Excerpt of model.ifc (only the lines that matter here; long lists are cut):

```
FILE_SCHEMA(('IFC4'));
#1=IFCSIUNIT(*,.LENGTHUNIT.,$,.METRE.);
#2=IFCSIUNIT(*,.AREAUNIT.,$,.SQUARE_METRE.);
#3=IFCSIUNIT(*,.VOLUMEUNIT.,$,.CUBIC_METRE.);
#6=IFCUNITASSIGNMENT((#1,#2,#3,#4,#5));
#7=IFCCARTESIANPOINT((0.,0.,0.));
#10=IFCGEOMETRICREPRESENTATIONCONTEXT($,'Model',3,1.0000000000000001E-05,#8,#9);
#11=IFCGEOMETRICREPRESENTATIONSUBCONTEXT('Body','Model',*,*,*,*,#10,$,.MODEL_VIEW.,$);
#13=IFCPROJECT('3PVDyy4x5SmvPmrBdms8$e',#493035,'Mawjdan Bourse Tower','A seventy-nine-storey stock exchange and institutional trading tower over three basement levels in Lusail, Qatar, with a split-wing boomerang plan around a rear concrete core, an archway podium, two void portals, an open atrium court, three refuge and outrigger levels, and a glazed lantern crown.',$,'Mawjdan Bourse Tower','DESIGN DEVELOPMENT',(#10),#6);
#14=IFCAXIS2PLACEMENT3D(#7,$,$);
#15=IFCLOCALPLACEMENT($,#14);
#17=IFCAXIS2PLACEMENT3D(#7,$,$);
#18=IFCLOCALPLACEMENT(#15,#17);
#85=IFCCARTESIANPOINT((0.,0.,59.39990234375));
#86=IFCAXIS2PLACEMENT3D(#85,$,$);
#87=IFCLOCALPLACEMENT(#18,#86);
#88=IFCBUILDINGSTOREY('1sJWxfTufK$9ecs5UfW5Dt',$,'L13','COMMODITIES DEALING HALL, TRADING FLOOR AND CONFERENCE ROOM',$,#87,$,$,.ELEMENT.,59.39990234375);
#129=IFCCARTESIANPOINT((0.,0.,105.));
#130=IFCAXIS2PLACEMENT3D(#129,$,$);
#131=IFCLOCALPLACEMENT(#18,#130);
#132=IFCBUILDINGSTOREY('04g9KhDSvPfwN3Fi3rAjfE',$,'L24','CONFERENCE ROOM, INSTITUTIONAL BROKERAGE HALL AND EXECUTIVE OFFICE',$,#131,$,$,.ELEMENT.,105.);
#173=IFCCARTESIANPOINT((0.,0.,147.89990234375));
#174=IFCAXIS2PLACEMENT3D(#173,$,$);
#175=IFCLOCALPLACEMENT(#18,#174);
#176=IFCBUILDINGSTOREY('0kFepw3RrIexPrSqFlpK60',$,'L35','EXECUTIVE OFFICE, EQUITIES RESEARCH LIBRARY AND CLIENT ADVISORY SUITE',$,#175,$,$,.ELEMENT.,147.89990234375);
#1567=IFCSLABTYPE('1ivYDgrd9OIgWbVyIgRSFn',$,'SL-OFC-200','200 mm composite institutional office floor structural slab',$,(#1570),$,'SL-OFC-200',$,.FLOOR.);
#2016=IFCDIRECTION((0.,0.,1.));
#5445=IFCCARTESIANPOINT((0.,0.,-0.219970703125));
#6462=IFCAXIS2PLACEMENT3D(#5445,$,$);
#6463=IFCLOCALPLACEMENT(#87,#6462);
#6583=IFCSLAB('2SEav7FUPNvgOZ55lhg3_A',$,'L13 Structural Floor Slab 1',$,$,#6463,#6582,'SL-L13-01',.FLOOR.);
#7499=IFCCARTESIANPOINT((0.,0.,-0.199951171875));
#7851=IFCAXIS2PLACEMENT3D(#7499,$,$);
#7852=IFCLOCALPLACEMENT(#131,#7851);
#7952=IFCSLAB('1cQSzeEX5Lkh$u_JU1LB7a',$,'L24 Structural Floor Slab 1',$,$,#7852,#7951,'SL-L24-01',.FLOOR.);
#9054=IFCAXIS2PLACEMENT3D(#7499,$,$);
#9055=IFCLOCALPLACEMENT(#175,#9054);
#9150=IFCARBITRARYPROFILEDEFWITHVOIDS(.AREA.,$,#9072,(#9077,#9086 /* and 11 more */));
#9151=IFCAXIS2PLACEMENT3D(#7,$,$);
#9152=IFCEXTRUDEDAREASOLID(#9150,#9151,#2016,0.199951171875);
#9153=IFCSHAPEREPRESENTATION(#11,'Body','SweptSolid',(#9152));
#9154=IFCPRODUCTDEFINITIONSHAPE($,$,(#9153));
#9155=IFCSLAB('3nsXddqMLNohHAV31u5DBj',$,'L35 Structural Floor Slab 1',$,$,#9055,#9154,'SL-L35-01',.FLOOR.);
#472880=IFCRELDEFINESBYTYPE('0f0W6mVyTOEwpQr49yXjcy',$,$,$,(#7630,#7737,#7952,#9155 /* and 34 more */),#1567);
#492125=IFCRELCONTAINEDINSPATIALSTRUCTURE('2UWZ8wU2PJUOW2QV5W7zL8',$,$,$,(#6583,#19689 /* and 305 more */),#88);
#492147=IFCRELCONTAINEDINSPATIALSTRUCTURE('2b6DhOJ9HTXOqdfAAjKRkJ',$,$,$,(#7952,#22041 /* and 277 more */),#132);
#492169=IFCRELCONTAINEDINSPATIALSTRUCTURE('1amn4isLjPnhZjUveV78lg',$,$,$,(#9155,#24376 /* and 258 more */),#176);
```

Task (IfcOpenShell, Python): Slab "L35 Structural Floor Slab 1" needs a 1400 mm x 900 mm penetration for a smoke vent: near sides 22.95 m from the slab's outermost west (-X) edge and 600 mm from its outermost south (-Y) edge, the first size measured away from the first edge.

```python
import numpy as np
import ifcopenshell
import ifcopenshell.api.feature
import ifcopenshell.api.geometry
import ifcopenshell.api.root
import ifcopenshell.geom
import ifcopenshell.util.placement
import ifcopenshell.util.representation
import ifcopenshell.util.shape
import ifcopenshell.util.unit

model = ifcopenshell.open("model.ifc")
unit_scale = ifcopenshell.util.unit.calculate_unit_scale(model)
settings = ifcopenshell.geom.settings()


def volume(element):
    """Net volume in cubic metres, openings subtracted."""
    shape = ifcopenshell.geom.create_shape(settings, element)
    return ifcopenshell.util.shape.get_volume(shape.geometry)


slab = model.by_id(9155)
before = volume(slab)

# Extent in the slab's own axes, in metres. The edges named are its -X and -Y sides.
slab_shape = ifcopenshell.geom.create_shape(settings, slab)
vertices = ifcopenshell.util.shape.get_vertices(slab_shape.geometry)
x_min, y_min, bottom = vertices.min(axis=0)
top = vertices[:, 2].max()

opening = ifcopenshell.api.root.create_entity(model, ifc_class="IfcOpeningElement", name="Smoke vent opening", predefined_type="OPENING")
context = ifcopenshell.util.representation.get_context(model, "Model", "Body", "MODEL_VIEW")
width, depth = 1.4, 0.9
outline = [(0.0, 0.0), (width, 0.0), (width, depth), (0.0, depth), (0.0, 0.0)]
# Overshoot both faces by 50 mm so the cut is clean.
shape = ifcopenshell.api.geometry.add_slab_representation(
    model, context=context, depth=top - bottom + 0.1, polyline=outline
)
ifcopenshell.api.geometry.assign_representation(model, product=opening, representation=shape)

matrix = ifcopenshell.util.placement.get_local_placement(slab.ObjectPlacement)
matrix[:, 3] = matrix @ np.append(np.array([x_min + 22.95, y_min + 0.6, bottom - 0.05]) / unit_scale, 1.0)
ifcopenshell.api.geometry.edit_object_placement(model, product=opening, matrix=matrix, is_si=False)
ifcopenshell.api.feature.add_feature(model, feature=opening, element=slab)

after = volume(slab)

print(f"slab volume {before:.3f} -> {after:.3f} m3")

model.write("model_edited.ifc")
```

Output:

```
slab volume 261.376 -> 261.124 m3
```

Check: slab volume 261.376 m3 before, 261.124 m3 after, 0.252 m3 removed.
